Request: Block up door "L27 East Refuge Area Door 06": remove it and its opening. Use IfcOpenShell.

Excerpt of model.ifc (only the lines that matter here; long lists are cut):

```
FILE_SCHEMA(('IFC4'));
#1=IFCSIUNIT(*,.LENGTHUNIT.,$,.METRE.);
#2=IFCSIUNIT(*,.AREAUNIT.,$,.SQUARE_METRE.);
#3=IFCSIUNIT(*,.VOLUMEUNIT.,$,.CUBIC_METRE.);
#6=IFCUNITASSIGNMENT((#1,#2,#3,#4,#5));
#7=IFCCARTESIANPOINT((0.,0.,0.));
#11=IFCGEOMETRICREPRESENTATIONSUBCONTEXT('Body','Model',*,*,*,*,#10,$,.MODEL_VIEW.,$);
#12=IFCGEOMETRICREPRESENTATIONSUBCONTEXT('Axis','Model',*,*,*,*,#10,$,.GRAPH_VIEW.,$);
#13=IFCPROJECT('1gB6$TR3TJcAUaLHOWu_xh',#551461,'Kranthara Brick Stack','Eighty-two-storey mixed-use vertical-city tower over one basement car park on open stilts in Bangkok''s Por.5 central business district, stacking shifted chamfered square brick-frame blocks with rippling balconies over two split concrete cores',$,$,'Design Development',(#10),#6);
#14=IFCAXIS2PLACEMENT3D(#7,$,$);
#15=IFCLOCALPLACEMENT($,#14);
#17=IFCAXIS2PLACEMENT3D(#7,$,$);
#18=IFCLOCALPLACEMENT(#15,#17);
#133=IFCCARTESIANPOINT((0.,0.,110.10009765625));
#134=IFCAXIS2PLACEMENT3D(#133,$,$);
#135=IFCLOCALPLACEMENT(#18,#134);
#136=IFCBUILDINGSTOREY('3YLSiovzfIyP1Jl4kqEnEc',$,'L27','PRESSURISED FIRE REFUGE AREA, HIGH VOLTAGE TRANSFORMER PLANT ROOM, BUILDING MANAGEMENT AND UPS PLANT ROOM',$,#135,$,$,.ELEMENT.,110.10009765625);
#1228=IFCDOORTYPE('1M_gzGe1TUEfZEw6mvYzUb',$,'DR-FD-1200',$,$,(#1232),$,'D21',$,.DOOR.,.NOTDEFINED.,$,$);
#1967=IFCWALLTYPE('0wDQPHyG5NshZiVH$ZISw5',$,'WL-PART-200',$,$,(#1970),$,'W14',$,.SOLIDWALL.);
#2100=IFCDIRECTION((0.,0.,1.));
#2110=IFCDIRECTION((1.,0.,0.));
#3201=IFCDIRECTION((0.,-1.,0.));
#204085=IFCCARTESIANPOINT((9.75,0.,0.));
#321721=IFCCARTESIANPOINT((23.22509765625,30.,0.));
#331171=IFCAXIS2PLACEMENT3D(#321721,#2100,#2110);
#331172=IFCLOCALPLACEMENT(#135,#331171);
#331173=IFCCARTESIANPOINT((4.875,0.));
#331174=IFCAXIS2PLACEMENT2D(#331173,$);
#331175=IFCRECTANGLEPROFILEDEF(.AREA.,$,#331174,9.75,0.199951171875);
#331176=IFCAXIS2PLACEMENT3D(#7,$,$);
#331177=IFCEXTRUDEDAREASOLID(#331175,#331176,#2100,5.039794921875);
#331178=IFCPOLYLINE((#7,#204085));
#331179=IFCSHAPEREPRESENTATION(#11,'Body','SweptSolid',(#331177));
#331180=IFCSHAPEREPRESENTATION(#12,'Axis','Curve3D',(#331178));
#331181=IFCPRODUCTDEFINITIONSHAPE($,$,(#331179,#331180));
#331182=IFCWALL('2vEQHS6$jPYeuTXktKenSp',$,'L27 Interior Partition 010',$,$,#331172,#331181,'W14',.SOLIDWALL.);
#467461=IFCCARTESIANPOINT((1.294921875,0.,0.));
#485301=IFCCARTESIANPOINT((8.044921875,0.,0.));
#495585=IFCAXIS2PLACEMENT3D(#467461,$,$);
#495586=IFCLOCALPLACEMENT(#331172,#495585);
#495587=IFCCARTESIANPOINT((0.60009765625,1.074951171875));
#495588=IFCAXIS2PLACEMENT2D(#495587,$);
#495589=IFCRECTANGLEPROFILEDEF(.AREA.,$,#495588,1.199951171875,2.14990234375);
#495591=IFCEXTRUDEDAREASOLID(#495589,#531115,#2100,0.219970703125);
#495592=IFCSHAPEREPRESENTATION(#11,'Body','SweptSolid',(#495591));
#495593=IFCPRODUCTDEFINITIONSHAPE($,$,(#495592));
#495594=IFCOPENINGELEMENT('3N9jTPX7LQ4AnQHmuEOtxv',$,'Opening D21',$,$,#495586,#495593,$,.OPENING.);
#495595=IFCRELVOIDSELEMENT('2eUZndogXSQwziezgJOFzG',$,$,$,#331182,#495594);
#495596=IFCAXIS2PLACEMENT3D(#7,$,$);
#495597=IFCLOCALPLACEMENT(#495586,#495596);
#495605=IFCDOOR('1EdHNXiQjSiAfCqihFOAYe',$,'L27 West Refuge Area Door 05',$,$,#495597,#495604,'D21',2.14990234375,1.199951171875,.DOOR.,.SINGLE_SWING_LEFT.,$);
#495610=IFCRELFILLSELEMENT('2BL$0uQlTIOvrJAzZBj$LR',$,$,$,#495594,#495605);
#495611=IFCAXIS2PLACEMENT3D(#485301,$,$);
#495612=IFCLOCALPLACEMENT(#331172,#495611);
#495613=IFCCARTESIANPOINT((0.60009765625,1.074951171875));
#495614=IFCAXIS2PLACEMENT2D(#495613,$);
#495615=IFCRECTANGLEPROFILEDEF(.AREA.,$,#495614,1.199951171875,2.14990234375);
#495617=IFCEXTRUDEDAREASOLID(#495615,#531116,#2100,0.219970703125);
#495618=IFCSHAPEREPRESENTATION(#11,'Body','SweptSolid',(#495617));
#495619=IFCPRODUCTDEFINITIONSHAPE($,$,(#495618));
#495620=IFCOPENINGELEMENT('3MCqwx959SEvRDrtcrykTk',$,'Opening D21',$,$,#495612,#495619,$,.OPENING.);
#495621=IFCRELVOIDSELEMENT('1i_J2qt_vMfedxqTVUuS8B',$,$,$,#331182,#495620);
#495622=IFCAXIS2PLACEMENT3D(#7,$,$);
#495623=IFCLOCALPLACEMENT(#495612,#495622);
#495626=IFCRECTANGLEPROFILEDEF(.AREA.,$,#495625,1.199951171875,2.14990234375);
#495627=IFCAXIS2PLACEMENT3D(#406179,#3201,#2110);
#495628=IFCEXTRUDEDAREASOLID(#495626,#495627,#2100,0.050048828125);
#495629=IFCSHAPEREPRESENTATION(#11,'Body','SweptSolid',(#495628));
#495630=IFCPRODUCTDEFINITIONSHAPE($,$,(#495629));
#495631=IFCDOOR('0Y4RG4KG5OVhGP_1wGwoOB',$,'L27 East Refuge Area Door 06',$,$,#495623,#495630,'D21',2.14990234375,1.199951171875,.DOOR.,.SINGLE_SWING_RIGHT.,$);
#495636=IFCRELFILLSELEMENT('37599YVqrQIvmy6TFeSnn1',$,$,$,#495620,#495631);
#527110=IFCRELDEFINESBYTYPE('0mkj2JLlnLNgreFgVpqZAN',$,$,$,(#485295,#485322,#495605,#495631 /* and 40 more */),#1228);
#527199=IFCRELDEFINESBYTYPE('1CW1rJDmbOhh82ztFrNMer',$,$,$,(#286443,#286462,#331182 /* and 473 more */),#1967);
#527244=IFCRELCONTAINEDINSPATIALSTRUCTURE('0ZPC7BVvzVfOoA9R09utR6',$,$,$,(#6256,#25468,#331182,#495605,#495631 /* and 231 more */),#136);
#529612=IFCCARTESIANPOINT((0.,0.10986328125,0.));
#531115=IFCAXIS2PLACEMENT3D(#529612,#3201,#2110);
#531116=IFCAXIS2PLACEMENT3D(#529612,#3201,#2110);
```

```python
import ifcopenshell
import ifcopenshell.api.feature
import ifcopenshell.api.root
import ifcopenshell.geom
import ifcopenshell.util.shape

model = ifcopenshell.open("model.ifc")
settings = ifcopenshell.geom.settings()


def volume(element):
    """Net volume in cubic metres, openings subtracted."""
    shape = ifcopenshell.geom.create_shape(settings, element)
    return ifcopenshell.util.shape.get_volume(shape.geometry)


door = model.by_guid("0Y4RG4KG5OVhGP_1wGwoOB")
opening = door.FillsVoids[0].RelatingOpeningElement
wall = opening.VoidsElements[0].RelatingBuildingElement
before = volume(wall)

ifcopenshell.api.root.remove_product(model, product=door)
ifcopenshell.api.feature.remove_feature(model, feature=opening)

after = volume(wall)

print(f"wall volume {before:.3f} -> {after:.3f} m3")

model.write("model_edited.ifc")
```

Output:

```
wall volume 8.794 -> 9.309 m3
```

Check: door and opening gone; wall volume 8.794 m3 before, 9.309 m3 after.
